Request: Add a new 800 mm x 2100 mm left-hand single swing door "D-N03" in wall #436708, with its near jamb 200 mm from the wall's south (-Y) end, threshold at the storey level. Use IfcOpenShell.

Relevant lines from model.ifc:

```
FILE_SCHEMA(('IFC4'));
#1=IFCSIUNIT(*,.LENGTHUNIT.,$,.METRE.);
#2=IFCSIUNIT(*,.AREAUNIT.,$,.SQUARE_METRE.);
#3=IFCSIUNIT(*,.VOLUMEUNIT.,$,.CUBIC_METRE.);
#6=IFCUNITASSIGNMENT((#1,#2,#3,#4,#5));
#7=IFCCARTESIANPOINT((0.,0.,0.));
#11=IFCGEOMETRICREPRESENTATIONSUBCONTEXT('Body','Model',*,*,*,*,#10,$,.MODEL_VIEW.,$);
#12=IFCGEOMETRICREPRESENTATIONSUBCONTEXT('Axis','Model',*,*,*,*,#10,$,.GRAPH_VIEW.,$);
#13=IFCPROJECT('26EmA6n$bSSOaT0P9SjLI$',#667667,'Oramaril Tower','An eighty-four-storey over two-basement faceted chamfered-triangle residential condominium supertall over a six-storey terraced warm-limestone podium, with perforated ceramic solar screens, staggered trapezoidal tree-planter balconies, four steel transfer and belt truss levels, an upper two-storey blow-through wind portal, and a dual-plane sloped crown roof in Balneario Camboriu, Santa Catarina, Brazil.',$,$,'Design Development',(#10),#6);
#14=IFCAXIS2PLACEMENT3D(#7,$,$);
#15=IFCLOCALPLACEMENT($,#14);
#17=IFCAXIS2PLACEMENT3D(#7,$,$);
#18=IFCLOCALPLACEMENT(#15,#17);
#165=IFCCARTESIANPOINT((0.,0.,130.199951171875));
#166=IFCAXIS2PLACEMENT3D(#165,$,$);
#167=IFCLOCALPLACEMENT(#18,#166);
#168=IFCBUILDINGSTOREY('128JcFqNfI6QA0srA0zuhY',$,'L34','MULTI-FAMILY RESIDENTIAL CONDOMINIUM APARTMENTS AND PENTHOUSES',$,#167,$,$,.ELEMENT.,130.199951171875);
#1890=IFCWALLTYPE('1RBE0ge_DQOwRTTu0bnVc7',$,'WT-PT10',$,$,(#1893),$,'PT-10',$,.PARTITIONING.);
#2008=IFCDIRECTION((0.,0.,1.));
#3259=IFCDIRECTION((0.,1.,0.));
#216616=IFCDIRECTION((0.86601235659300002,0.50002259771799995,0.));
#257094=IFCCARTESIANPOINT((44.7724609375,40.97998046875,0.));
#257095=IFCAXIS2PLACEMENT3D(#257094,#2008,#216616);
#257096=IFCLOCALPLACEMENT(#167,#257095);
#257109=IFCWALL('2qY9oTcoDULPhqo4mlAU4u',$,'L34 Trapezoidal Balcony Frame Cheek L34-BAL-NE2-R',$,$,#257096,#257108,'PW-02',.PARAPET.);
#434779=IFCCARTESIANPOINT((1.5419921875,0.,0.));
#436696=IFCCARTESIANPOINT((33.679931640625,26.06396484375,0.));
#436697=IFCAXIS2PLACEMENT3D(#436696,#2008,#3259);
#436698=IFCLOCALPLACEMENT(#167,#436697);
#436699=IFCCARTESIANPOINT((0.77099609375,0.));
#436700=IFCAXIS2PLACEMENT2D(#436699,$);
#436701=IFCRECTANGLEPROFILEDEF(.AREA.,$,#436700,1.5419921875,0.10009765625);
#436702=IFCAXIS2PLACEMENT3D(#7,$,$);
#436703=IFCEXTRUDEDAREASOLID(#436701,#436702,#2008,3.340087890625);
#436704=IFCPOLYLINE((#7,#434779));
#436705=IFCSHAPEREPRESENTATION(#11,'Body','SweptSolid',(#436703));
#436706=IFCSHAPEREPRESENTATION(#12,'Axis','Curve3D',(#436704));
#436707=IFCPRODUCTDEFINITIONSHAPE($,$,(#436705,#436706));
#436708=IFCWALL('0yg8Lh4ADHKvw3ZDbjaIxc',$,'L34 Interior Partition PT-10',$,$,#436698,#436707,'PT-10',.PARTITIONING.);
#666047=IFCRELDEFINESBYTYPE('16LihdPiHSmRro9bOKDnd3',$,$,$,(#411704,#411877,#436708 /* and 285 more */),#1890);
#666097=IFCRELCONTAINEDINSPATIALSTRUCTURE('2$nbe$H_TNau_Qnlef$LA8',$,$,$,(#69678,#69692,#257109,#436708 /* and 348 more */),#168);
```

```python
import numpy as np
import ifcopenshell
import ifcopenshell.api.feature
import ifcopenshell.api.geometry
import ifcopenshell.api.root
import ifcopenshell.api.spatial
import ifcopenshell.geom
import ifcopenshell.util.element
import ifcopenshell.util.placement
import ifcopenshell.util.representation
import ifcopenshell.util.shape
import ifcopenshell.util.unit

model = ifcopenshell.open("model.ifc")
unit_scale = ifcopenshell.util.unit.calculate_unit_scale(model)
settings = ifcopenshell.geom.settings()


def volume(element):
    """Net volume in cubic metres, openings subtracted."""
    shape = ifcopenshell.geom.create_shape(settings, element)
    return ifcopenshell.util.shape.get_volume(shape.geometry)


wall = model.by_id(436708)
storey = ifcopenshell.util.element.get_container(wall, ifc_class="IfcBuildingStorey")
context = ifcopenshell.util.representation.get_context(model, "Model", "Body", "MODEL_VIEW")
before = volume(wall)

width, height, from_end, sill = 0.8, 2.1, 0.2, 0.0  # metres

# The wall runs along its own X axis, and the end named is its -X end.
wall_shape = ifcopenshell.geom.create_shape(settings, wall)
x, y, z = ifcopenshell.util.shape.get_vertices(wall_shape.geometry).T
start = x.min() + from_end
face, thickness = float(y.min()), float(y.max() - y.min())
wall_matrix = ifcopenshell.util.placement.get_local_placement(wall.ObjectPlacement)
level = ifcopenshell.util.placement.get_local_placement(storey.ObjectPlacement)[2, 3]


def in_wall(x, y):
    """Placement at x, y metres in the wall's axes, at sill height."""
    matrix = wall_matrix.copy()
    matrix[:, 3] = wall_matrix @ np.array([x / unit_scale, y / unit_scale, 0.0, 1.0])
    matrix[2, 3] = level + sill / unit_scale
    return matrix


# Opening: a box that overshoots both wall faces by 50 mm.
opening = ifcopenshell.api.root.create_entity(model, ifc_class="IfcOpeningElement", predefined_type="OPENING")
box = ifcopenshell.api.geometry.add_wall_representation(
    model, context=context, length=width, height=height, thickness=thickness + 0.1
)
ifcopenshell.api.geometry.assign_representation(model, product=opening, representation=box)
ifcopenshell.api.geometry.edit_object_placement(model, product=opening, matrix=in_wall(start, face - 0.05), is_si=False)
ifcopenshell.api.feature.add_feature(model, feature=opening, element=wall)

door = ifcopenshell.api.root.create_entity(model, ifc_class="IfcDoor", name="D-N03", predefined_type="DOOR")
door.OverallWidth, door.OverallHeight = width / unit_scale, height / unit_scale
door.OperationType = "SINGLE_SWING_LEFT"
body = ifcopenshell.api.geometry.add_door_representation(
    model,
    context=context,
    overall_width=door.OverallWidth,
    overall_height=door.OverallHeight,
    operation_type="SINGLE_SWING_LEFT",
    lining_properties={"LiningDepth": thickness / unit_scale, "ThresholdDepth": thickness / unit_scale},
)
ifcopenshell.api.geometry.assign_representation(model, product=door, representation=body)
ifcopenshell.api.spatial.assign_container(model, products=[door], relating_structure=storey)
ifcopenshell.api.feature.add_filling(model, opening=opening, element=door)

# The lining spans the wall, so the door starts at the wall face.
ifcopenshell.api.geometry.edit_object_placement(model, product=door, matrix=in_wall(start, face), is_si=False)

after = volume(wall)

print(f"wall volume {before:.3f} -> {after:.3f} m3")

model.write("model_edited.ifc")
```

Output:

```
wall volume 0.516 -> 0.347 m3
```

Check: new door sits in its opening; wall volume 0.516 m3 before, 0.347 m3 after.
